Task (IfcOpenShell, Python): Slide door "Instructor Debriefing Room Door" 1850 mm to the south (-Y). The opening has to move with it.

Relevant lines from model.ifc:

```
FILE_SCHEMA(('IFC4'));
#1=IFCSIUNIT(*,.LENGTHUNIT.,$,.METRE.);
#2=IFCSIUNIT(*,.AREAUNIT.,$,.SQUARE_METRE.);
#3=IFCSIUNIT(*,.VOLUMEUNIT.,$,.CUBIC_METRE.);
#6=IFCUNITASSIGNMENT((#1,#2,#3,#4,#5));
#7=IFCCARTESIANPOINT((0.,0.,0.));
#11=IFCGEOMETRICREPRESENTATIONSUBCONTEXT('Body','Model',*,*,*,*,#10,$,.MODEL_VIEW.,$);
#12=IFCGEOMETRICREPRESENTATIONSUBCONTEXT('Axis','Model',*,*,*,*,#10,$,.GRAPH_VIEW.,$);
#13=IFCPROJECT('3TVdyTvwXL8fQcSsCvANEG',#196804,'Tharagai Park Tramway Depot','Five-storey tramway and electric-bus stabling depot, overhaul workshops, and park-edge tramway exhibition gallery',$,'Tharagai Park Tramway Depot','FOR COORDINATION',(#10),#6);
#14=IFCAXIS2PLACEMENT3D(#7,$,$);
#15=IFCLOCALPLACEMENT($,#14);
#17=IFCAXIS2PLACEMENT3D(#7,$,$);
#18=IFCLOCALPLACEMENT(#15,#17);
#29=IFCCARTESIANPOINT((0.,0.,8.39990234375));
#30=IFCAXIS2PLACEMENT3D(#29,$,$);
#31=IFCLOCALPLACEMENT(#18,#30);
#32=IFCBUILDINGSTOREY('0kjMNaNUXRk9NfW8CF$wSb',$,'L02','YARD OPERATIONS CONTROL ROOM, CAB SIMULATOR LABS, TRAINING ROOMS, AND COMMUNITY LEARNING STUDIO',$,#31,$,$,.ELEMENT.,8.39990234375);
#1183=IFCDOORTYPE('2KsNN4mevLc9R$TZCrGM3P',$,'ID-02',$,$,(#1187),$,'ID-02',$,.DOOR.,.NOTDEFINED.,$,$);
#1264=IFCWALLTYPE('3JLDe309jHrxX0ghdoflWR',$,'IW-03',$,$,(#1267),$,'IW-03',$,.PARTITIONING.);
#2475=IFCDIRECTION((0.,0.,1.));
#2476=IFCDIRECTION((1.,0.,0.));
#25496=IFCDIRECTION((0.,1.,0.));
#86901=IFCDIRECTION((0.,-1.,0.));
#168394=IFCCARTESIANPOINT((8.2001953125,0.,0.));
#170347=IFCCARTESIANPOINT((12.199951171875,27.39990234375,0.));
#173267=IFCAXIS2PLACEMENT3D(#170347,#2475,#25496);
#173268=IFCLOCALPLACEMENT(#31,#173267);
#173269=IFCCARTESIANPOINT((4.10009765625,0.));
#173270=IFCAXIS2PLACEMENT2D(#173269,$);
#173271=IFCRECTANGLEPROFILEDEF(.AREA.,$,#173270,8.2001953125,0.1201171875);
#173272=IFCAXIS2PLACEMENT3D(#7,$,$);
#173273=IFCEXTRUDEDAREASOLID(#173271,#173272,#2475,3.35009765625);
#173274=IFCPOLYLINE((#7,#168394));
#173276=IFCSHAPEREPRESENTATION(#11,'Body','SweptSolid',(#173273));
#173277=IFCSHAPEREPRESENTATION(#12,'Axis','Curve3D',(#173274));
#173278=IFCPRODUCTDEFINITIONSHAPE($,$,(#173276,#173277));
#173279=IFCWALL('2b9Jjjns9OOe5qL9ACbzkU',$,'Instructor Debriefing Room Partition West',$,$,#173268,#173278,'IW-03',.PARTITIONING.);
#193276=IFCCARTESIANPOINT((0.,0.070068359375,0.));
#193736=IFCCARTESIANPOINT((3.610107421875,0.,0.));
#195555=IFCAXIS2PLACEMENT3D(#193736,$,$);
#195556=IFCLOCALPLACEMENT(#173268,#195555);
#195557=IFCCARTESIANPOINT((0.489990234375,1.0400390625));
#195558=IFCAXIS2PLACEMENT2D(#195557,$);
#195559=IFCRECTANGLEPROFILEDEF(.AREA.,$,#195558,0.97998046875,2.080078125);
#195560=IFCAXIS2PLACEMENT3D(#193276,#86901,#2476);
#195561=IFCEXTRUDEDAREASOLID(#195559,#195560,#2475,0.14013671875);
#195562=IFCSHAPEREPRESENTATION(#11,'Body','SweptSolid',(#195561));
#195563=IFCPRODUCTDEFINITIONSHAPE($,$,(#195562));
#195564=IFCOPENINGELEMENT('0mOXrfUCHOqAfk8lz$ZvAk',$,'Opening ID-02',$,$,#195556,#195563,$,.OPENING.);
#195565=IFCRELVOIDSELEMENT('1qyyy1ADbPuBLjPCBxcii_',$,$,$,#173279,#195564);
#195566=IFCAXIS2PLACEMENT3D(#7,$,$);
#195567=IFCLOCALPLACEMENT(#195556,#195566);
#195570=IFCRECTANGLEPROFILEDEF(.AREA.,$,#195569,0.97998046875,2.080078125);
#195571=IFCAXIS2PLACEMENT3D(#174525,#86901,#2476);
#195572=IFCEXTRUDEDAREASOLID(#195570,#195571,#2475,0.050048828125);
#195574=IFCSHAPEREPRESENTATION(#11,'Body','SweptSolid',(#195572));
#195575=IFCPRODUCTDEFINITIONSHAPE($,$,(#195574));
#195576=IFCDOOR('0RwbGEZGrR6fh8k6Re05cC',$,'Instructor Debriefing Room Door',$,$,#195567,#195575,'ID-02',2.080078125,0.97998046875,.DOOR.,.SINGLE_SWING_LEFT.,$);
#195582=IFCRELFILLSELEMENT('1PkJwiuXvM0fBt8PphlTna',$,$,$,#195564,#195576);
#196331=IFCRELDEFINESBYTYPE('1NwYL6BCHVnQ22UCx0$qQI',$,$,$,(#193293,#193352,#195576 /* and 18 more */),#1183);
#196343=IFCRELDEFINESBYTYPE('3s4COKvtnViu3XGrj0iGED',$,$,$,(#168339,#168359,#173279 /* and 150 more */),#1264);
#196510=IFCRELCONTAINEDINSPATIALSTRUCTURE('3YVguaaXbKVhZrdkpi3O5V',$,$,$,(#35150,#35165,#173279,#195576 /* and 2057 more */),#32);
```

```python
import ifcopenshell
import ifcopenshell.api.geometry
import ifcopenshell.util.placement

model = ifcopenshell.open("model.ifc")

door = model.by_guid("0RwbGEZGrR6fh8k6Re05cC")
opening = door.FillsVoids[0].RelatingOpeningElement
wall = opening.VoidsElements[0].RelatingBuildingElement

wall_matrix = ifcopenshell.util.placement.get_local_placement(wall.ObjectPlacement)
shift = wall_matrix[:3, 0] * -1.85
before = ifcopenshell.util.placement.get_local_placement(door.ObjectPlacement)[:3, 3].copy()

# The door is placed relative to its opening, so it follows when the opening moves.
matrix = ifcopenshell.util.placement.get_local_placement(opening.ObjectPlacement)
matrix[:3, 3] += shift
ifcopenshell.api.geometry.edit_object_placement(
    model, product=opening, matrix=matrix, is_si=False, should_transform_children=True
)

after = ifcopenshell.util.placement.get_local_placement(door.ObjectPlacement)[:3, 3]
print("door moved by", (after - before).round(3) + 0.0)

model.write("model-out.ifc")
```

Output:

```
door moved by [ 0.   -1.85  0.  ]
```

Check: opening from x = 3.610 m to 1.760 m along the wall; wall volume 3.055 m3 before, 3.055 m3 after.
